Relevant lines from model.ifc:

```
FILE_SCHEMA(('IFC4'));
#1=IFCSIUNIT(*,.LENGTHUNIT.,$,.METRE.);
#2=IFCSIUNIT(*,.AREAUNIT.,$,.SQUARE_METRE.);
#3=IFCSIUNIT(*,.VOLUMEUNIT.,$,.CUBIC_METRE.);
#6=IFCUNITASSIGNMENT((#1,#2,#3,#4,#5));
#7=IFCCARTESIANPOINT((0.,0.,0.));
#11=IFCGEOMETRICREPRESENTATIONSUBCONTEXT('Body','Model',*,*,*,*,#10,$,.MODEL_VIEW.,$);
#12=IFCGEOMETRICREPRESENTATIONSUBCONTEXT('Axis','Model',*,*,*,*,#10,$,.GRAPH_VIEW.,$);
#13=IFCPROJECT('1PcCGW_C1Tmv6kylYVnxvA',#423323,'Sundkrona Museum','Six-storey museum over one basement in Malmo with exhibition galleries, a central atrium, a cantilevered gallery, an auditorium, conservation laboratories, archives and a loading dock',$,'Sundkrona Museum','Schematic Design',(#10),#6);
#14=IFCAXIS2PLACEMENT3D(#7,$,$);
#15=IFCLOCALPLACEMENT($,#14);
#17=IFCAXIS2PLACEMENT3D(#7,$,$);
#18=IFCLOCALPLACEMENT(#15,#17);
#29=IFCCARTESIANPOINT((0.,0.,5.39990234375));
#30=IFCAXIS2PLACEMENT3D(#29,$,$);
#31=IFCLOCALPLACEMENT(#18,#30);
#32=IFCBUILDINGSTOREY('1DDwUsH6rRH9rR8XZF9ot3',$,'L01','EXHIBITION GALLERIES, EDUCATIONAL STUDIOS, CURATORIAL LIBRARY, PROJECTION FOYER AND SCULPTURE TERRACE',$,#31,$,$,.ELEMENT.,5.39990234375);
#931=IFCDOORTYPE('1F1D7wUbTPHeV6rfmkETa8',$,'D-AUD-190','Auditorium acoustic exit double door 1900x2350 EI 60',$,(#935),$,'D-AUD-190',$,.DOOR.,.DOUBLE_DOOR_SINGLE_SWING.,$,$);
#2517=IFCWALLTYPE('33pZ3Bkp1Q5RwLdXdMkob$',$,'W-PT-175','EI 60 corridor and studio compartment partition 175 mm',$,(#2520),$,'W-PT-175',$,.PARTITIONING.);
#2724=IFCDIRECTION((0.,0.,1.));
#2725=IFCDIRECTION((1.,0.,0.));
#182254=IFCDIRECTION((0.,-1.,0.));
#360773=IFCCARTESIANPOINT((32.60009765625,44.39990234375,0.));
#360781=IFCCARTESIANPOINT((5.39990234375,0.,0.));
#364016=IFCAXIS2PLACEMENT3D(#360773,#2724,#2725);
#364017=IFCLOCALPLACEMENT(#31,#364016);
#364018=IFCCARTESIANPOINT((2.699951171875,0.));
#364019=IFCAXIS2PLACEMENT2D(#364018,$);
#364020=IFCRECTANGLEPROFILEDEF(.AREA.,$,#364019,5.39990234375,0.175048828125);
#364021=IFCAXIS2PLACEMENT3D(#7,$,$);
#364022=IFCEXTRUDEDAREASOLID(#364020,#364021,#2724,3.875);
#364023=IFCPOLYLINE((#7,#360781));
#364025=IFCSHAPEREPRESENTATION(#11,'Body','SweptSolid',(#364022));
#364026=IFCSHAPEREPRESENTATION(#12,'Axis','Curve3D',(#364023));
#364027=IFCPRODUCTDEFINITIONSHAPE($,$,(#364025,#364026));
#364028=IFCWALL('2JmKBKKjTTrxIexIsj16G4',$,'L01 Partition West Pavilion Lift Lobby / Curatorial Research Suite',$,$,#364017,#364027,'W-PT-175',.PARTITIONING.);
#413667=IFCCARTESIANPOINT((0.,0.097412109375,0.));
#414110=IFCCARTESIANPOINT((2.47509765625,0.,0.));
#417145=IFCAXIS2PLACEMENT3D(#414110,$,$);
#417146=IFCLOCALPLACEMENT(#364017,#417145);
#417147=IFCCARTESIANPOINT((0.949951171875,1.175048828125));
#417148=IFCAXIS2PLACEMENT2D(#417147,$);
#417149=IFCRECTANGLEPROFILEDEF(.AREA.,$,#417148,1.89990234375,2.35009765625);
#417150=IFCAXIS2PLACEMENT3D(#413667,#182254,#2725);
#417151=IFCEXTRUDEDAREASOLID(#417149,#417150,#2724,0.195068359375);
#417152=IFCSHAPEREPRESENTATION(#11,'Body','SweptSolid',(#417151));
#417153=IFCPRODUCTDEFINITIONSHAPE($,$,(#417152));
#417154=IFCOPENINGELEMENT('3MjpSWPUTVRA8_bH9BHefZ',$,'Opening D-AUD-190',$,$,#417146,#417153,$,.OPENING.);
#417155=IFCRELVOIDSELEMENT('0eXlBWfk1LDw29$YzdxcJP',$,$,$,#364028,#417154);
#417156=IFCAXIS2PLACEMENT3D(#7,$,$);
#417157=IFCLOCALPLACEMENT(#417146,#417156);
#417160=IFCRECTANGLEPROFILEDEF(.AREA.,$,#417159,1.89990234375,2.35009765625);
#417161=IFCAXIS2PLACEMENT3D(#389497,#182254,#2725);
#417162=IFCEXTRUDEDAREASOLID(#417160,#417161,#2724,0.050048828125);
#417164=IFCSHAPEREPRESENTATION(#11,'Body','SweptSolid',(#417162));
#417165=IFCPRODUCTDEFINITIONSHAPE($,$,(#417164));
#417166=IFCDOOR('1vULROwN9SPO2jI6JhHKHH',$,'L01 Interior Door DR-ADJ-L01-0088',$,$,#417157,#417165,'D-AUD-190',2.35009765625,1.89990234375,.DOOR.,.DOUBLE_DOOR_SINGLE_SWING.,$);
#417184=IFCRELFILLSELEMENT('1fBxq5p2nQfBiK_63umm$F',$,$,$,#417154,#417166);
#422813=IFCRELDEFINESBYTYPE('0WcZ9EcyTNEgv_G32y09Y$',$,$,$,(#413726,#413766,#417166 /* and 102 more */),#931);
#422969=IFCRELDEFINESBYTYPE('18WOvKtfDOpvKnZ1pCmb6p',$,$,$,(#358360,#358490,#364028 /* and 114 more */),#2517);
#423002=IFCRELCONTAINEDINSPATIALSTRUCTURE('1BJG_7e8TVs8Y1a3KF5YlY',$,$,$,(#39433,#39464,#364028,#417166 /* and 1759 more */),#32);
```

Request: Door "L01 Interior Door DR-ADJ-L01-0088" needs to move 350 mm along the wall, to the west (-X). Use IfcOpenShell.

```python
import ifcopenshell
import ifcopenshell.api.geometry
import ifcopenshell.util.placement

model = ifcopenshell.open("model.ifc")

door = model.by_id(417166)
opening = door.FillsVoids[0].RelatingOpeningElement
wall = opening.VoidsElements[0].RelatingBuildingElement

wall_matrix = ifcopenshell.util.placement.get_local_placement(wall.ObjectPlacement)
shift = wall_matrix[:3, 0] * -0.35
before = ifcopenshell.util.placement.get_local_placement(door.ObjectPlacement)[:3, 3].copy()

# The door is placed relative to its opening, so it follows when the opening moves.
matrix = ifcopenshell.util.placement.get_local_placement(opening.ObjectPlacement)
matrix[:3, 3] += shift
ifcopenshell.api.geometry.edit_object_placement(
    model, product=opening, matrix=matrix, is_si=False, should_transform_children=True
)

after = ifcopenshell.util.placement.get_local_placement(door.ObjectPlacement)[:3, 3]
print("door moved by", (after - before).round(3) + 0.0)

model.write("model_rev.ifc")
```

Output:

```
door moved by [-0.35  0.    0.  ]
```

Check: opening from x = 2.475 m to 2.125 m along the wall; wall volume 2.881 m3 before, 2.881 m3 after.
